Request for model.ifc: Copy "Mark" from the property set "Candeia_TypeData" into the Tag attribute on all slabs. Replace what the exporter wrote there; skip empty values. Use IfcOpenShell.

First a look at what the model holds.

```python
import ifcopenshell
import ifcopenshell.util.element

model = ifcopenshell.open("model.ifc")
print(model.schema)
slabs = model.by_type("IfcSlab")
print(len(slabs), "slabs")
for e in slabs[:8]:
    source = ifcopenshell.util.element.get_pset(e, "Candeia_TypeData", "Mark")
    target = e.Tag
    print(e.id(), repr(source), repr(target), sep=" | ")
```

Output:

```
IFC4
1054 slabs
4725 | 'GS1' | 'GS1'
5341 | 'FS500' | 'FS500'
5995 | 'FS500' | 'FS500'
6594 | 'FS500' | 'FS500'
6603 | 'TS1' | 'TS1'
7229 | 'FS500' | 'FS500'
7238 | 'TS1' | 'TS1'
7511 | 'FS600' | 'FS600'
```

```python
import ifcopenshell
import ifcopenshell.util.element

model = ifcopenshell.open("model.ifc")

count = 0
for e in model.by_type("IfcSlab"):
    value = ifcopenshell.util.element.get_pset(e, "Candeia_TypeData", "Mark")
    current = e.Tag
    if not value or not value.strip() or current == value:
        continue
    e.Tag = value
    count += 1

print(count, "slabs updated")

model.write("model_updated.ifc")
```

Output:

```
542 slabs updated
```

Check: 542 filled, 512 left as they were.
